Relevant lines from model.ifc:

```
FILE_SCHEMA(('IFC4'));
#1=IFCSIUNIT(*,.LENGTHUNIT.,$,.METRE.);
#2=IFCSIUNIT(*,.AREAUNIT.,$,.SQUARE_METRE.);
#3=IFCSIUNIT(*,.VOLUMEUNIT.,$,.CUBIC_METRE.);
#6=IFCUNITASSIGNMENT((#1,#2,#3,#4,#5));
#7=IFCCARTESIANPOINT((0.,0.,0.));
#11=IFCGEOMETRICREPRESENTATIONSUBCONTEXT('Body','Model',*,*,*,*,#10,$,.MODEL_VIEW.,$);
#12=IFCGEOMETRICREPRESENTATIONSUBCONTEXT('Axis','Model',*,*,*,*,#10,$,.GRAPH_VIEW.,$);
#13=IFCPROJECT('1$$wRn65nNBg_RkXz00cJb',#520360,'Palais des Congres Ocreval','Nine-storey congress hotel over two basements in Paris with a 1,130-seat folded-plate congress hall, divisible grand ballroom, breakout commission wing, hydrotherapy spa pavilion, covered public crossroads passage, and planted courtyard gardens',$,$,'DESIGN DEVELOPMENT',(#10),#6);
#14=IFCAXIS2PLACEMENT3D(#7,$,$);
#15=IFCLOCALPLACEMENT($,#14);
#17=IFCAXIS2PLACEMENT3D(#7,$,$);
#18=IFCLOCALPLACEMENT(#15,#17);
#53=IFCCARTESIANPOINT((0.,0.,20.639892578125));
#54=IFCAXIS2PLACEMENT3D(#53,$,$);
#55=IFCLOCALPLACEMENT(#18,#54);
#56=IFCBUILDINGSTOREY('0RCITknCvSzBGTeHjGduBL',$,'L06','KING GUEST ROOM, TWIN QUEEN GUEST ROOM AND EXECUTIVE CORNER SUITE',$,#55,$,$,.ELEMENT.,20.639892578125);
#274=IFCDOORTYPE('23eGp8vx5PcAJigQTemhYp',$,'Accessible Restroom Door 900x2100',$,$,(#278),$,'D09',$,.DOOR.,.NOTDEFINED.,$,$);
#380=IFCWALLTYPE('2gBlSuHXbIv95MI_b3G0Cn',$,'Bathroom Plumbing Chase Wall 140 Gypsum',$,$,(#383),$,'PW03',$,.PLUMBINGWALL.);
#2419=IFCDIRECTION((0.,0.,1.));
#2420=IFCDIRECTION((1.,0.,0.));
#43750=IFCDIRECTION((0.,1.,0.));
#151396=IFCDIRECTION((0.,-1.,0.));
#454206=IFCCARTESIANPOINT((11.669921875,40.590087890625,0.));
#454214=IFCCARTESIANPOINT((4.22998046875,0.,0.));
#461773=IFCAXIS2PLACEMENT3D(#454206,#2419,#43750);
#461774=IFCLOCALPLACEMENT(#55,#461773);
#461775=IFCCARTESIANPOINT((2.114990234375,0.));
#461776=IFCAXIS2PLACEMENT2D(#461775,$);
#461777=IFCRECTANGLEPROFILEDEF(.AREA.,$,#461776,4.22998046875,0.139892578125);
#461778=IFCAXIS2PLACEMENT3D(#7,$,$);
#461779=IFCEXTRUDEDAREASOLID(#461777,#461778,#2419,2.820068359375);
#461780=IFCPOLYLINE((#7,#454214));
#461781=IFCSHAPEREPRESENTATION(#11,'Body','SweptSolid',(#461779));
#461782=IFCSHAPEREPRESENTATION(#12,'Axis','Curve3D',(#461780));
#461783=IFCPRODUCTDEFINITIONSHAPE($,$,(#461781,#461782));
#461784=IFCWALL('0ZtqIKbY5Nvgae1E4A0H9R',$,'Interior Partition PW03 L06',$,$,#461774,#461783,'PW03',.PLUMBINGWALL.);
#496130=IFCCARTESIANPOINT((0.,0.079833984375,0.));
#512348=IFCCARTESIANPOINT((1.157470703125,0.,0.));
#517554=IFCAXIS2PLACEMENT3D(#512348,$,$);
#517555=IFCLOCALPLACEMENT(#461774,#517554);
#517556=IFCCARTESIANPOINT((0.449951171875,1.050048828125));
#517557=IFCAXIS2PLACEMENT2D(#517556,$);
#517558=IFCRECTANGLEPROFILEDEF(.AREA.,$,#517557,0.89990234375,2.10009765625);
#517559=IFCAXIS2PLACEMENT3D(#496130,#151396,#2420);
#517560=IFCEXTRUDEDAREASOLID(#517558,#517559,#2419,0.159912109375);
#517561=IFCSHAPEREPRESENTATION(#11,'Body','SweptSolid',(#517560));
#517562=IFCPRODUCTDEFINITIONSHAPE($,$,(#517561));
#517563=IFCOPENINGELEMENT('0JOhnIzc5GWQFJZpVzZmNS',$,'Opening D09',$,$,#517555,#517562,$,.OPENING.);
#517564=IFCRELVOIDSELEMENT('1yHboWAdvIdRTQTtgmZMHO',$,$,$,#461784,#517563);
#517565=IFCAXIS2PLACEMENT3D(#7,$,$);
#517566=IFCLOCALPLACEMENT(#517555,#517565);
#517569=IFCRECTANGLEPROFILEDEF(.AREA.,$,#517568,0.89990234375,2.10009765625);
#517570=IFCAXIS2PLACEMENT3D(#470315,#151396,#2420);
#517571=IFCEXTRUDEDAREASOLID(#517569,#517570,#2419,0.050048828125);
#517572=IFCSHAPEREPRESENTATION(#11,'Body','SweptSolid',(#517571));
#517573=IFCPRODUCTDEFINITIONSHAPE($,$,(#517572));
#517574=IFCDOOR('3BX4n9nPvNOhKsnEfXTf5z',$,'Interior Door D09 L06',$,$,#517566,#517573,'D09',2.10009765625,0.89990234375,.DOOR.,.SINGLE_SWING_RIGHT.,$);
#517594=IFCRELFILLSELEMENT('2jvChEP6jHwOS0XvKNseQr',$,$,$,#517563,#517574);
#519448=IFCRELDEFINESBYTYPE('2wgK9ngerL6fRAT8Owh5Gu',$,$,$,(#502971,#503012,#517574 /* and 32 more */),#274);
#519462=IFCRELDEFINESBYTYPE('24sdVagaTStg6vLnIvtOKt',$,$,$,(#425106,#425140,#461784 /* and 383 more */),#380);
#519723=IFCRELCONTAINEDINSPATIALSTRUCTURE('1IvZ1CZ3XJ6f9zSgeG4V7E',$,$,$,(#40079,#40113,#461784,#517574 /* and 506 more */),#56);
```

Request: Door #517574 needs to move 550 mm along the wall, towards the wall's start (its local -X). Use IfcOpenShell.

```python
import ifcopenshell
import ifcopenshell.api.geometry
import ifcopenshell.util.placement
import ifcopenshell.util.unit

model = ifcopenshell.open("model.ifc")
unit_scale = ifcopenshell.util.unit.calculate_unit_scale(model)

door = model.by_guid("3BX4n9nPvNOhKsnEfXTf5z")
opening = door.FillsVoids[0].RelatingOpeningElement
wall = opening.VoidsElements[0].RelatingBuildingElement

wall_matrix = ifcopenshell.util.placement.get_local_placement(wall.ObjectPlacement)
shift = wall_matrix[:3, 0] * -0.55 / unit_scale
before = ifcopenshell.util.placement.get_local_placement(door.ObjectPlacement)[:3, 3].copy()

# The door is placed relative to its opening, so it follows when the opening moves.
matrix = ifcopenshell.util.placement.get_local_placement(opening.ObjectPlacement)
matrix[:3, 3] += shift
ifcopenshell.api.geometry.edit_object_placement(
    model, product=opening, matrix=matrix, is_si=False, should_transform_children=True
)

after = ifcopenshell.util.placement.get_local_placement(door.ObjectPlacement)[:3, 3]
print("door moved by", (after - before).round(3) + 0.0)

model.write("model_rev.ifc")
```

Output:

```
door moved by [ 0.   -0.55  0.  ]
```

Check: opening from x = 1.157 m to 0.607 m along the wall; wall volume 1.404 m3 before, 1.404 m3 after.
